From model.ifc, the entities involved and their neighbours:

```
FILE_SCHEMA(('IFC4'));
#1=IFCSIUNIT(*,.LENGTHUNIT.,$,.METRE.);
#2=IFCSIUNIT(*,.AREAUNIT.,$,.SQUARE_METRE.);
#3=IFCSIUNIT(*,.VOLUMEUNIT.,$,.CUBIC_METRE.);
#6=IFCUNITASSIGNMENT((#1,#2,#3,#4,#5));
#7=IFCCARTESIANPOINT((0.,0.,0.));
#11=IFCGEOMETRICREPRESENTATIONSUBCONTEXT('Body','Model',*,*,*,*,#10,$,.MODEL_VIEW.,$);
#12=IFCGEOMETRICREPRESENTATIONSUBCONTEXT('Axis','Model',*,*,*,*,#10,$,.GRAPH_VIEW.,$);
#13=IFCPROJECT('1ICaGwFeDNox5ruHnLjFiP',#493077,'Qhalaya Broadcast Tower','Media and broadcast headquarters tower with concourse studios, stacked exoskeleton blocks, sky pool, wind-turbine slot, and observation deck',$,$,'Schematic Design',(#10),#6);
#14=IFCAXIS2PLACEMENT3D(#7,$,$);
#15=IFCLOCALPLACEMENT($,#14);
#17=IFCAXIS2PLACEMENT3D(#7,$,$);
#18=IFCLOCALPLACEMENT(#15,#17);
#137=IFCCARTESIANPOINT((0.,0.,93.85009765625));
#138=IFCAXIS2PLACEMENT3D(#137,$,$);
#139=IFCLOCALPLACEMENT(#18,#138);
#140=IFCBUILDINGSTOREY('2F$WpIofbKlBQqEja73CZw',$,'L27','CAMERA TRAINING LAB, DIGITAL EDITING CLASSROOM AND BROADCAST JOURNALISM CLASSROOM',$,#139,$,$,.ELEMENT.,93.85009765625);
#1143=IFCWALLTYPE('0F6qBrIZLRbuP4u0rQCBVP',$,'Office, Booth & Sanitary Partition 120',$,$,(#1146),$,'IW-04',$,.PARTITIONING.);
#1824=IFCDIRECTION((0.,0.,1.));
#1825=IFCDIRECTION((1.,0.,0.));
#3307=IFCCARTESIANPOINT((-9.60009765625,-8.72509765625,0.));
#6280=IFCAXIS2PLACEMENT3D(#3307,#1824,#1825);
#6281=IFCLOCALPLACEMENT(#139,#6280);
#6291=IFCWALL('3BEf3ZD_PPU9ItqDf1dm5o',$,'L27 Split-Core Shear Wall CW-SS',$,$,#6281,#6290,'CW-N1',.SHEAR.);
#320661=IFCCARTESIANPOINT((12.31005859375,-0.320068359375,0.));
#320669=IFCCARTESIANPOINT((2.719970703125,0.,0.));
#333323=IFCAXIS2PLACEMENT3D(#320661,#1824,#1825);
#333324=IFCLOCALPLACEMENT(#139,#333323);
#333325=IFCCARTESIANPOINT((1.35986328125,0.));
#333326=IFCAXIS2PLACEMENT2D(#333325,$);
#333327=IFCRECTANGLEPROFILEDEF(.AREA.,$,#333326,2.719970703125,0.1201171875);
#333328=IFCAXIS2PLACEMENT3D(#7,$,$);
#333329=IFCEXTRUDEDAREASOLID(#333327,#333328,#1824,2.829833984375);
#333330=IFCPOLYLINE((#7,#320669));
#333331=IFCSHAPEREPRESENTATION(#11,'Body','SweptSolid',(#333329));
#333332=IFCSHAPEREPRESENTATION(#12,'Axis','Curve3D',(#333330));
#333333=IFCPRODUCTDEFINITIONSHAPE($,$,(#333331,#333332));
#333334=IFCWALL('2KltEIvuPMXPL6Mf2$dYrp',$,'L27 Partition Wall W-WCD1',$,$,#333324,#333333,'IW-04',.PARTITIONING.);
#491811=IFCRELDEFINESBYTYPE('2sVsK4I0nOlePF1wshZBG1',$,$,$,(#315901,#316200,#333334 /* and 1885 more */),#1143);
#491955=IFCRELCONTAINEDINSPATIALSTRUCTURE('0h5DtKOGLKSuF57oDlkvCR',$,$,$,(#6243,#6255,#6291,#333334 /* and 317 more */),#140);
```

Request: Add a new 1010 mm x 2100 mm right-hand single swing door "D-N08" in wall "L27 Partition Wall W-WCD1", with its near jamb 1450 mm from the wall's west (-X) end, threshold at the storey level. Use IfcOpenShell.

```python
import numpy as np
import ifcopenshell
import ifcopenshell.api.feature
import ifcopenshell.api.geometry
import ifcopenshell.api.root
import ifcopenshell.api.spatial
import ifcopenshell.geom
import ifcopenshell.util.element
import ifcopenshell.util.placement
import ifcopenshell.util.representation
import ifcopenshell.util.shape
import ifcopenshell.util.unit

model = ifcopenshell.open("model.ifc")
unit_scale = ifcopenshell.util.unit.calculate_unit_scale(model)
settings = ifcopenshell.geom.settings()


def volume(element):
    """Net volume in cubic metres, openings subtracted."""
    shape = ifcopenshell.geom.create_shape(settings, element)
    return ifcopenshell.util.shape.get_volume(shape.geometry)


wall = model.by_guid("2KltEIvuPMXPL6Mf2$dYrp")
storey = ifcopenshell.util.element.get_container(wall, ifc_class="IfcBuildingStorey")
context = ifcopenshell.util.representation.get_context(model, "Model", "Body", "MODEL_VIEW")
before = volume(wall)

width, height, from_end, sill = 1.01, 2.1, 1.45, 0.0  # metres

# The wall runs along its own X axis, and the end named is its -X end.
wall_shape = ifcopenshell.geom.create_shape(settings, wall)
x, y, z = ifcopenshell.util.shape.get_vertices(wall_shape.geometry).T
start = x.min() + from_end
face, thickness = float(y.min()), float(y.max() - y.min())
wall_matrix = ifcopenshell.util.placement.get_local_placement(wall.ObjectPlacement)
level = ifcopenshell.util.placement.get_local_placement(storey.ObjectPlacement)[2, 3]


def in_wall(x, y):
    """Placement at x, y metres in the wall's axes, at sill height."""
    matrix = wall_matrix.copy()
    matrix[:, 3] = wall_matrix @ np.array([x / unit_scale, y / unit_scale, 0.0, 1.0])
    matrix[2, 3] = level + sill / unit_scale
    return matrix


# Opening: a box that overshoots both wall faces by 50 mm.
opening = ifcopenshell.api.root.create_entity(model, ifc_class="IfcOpeningElement", predefined_type="OPENING")
box = ifcopenshell.api.geometry.add_wall_representation(
    model, context=context, length=width, height=height, thickness=thickness + 0.1
)
ifcopenshell.api.geometry.assign_representation(model, product=opening, representation=box)
ifcopenshell.api.geometry.edit_object_placement(model, product=opening, matrix=in_wall(start, face - 0.05), is_si=False)
ifcopenshell.api.feature.add_feature(model, feature=opening, element=wall)

door = ifcopenshell.api.root.create_entity(model, ifc_class="IfcDoor", name="D-N08", predefined_type="DOOR")
door.OverallWidth, door.OverallHeight = width / unit_scale, height / unit_scale
door.OperationType = "SINGLE_SWING_RIGHT"
body = ifcopenshell.api.geometry.add_door_representation(
    model,
    context=context,
    overall_width=door.OverallWidth,
    overall_height=door.OverallHeight,
    operation_type="SINGLE_SWING_RIGHT",
    lining_properties={"LiningDepth": thickness / unit_scale, "ThresholdDepth": thickness / unit_scale},
)
ifcopenshell.api.geometry.assign_representation(model, product=door, representation=body)
ifcopenshell.api.spatial.assign_container(model, products=[door], relating_structure=storey)
ifcopenshell.api.feature.add_filling(model, opening=opening, element=door)

# The lining spans the wall, so the door starts at the wall face.
ifcopenshell.api.geometry.edit_object_placement(model, product=door, matrix=in_wall(start, face), is_si=False)

after = volume(wall)

print(f"wall volume {before:.3f} -> {after:.3f} m3")

model.write("model-out.ifc")
```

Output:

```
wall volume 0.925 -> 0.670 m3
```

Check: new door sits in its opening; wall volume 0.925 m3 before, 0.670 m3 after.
